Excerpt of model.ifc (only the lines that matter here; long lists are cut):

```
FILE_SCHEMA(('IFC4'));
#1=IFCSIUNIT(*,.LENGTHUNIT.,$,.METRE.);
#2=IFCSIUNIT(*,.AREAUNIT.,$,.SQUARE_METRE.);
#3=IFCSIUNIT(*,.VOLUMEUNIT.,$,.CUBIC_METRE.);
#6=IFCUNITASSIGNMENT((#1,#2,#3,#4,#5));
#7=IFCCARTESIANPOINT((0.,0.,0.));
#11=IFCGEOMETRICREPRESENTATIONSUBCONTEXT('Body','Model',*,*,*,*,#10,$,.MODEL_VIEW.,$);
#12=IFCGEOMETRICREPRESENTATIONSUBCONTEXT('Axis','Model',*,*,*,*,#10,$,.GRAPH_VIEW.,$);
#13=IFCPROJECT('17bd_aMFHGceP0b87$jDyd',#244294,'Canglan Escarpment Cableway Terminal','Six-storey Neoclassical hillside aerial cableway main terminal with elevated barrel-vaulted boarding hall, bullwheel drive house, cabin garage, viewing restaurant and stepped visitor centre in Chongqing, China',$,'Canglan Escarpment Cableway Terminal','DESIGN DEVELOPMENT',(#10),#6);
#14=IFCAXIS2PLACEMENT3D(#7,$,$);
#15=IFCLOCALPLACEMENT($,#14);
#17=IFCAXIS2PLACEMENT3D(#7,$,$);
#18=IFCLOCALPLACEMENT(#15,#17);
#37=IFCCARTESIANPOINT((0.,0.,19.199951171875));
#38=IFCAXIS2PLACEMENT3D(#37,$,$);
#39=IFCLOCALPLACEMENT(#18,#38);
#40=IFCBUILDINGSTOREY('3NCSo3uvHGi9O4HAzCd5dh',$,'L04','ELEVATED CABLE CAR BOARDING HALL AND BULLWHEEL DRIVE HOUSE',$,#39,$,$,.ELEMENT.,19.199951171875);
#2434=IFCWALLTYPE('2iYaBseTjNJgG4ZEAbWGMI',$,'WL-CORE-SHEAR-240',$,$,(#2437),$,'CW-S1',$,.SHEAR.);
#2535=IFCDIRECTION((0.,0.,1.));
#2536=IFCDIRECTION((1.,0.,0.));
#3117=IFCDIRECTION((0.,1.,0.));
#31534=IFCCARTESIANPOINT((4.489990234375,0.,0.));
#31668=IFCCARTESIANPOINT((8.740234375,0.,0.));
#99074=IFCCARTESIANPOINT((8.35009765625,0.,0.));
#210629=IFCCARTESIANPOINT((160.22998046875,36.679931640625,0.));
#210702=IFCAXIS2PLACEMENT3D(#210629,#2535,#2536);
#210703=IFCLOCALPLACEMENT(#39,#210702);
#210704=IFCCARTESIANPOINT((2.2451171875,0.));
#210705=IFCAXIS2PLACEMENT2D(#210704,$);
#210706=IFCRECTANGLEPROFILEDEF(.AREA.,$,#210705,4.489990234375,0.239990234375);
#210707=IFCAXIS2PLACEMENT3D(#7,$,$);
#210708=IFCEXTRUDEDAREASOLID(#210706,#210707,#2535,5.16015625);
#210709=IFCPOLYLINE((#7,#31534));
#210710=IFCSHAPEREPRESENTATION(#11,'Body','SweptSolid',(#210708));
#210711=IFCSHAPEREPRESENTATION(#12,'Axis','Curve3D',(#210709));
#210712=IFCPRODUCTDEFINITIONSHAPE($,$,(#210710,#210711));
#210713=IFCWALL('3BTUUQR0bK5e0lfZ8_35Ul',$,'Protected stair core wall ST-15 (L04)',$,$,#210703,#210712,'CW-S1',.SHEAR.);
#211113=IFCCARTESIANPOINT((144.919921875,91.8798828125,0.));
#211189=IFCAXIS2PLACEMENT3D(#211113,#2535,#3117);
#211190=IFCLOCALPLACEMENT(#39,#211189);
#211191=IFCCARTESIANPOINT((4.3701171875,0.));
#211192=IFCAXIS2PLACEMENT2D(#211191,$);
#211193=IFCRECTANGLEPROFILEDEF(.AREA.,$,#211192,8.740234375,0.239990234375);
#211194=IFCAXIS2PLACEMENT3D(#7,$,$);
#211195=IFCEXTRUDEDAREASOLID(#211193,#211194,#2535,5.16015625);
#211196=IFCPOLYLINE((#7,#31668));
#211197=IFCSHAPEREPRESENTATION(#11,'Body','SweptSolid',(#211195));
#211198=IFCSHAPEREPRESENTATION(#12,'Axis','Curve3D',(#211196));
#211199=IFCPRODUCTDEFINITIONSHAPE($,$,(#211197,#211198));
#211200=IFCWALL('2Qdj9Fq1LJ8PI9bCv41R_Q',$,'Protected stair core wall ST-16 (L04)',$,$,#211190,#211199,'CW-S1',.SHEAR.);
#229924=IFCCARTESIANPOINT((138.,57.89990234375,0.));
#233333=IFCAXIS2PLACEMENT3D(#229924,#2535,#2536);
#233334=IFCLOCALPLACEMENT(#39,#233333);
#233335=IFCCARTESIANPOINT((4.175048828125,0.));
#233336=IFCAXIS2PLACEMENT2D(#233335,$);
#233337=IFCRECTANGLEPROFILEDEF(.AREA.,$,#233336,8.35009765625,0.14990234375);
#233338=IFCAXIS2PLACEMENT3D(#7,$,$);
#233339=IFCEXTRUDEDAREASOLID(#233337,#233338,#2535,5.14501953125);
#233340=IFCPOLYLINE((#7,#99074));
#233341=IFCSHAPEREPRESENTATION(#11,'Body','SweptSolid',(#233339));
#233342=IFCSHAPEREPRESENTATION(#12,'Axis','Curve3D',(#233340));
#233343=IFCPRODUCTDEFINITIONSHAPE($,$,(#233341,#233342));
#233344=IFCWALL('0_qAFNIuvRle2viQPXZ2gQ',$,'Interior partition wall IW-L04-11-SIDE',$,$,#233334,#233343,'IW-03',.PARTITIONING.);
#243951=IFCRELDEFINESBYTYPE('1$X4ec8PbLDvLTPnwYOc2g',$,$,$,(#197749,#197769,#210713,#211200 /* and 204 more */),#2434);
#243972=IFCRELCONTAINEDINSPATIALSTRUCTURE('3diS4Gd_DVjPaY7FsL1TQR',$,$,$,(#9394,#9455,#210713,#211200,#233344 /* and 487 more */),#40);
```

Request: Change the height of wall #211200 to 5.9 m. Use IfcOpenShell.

```python
import ifcopenshell
import ifcopenshell.geom
import ifcopenshell.util.representation
import ifcopenshell.util.shape
import ifcopenshell.util.unit

model = ifcopenshell.open("model.ifc")
unit_scale = ifcopenshell.util.unit.calculate_unit_scale(model)
settings = ifcopenshell.geom.settings()


def volume(element):
    """Net volume in cubic metres, openings subtracted."""
    shape = ifcopenshell.geom.create_shape(settings, element)
    return ifcopenshell.util.shape.get_volume(shape.geometry)


wall = model.by_guid("2Qdj9Fq1LJ8PI9bCv41R_Q")
before = volume(wall)

body = ifcopenshell.util.representation.get_representation(wall, "Model", "Body")
solid = body.Items[0]
old_height = solid.Depth
solid.Depth = 5.9 / unit_scale
after = volume(wall)

print(f"height {old_height:g} -> {solid.Depth:g}, volume {before:.3f} -> {after:.3f} m3")

model.write("model_rev.ifc")
```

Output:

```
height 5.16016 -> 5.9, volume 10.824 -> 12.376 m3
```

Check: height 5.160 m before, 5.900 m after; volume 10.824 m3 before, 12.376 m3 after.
